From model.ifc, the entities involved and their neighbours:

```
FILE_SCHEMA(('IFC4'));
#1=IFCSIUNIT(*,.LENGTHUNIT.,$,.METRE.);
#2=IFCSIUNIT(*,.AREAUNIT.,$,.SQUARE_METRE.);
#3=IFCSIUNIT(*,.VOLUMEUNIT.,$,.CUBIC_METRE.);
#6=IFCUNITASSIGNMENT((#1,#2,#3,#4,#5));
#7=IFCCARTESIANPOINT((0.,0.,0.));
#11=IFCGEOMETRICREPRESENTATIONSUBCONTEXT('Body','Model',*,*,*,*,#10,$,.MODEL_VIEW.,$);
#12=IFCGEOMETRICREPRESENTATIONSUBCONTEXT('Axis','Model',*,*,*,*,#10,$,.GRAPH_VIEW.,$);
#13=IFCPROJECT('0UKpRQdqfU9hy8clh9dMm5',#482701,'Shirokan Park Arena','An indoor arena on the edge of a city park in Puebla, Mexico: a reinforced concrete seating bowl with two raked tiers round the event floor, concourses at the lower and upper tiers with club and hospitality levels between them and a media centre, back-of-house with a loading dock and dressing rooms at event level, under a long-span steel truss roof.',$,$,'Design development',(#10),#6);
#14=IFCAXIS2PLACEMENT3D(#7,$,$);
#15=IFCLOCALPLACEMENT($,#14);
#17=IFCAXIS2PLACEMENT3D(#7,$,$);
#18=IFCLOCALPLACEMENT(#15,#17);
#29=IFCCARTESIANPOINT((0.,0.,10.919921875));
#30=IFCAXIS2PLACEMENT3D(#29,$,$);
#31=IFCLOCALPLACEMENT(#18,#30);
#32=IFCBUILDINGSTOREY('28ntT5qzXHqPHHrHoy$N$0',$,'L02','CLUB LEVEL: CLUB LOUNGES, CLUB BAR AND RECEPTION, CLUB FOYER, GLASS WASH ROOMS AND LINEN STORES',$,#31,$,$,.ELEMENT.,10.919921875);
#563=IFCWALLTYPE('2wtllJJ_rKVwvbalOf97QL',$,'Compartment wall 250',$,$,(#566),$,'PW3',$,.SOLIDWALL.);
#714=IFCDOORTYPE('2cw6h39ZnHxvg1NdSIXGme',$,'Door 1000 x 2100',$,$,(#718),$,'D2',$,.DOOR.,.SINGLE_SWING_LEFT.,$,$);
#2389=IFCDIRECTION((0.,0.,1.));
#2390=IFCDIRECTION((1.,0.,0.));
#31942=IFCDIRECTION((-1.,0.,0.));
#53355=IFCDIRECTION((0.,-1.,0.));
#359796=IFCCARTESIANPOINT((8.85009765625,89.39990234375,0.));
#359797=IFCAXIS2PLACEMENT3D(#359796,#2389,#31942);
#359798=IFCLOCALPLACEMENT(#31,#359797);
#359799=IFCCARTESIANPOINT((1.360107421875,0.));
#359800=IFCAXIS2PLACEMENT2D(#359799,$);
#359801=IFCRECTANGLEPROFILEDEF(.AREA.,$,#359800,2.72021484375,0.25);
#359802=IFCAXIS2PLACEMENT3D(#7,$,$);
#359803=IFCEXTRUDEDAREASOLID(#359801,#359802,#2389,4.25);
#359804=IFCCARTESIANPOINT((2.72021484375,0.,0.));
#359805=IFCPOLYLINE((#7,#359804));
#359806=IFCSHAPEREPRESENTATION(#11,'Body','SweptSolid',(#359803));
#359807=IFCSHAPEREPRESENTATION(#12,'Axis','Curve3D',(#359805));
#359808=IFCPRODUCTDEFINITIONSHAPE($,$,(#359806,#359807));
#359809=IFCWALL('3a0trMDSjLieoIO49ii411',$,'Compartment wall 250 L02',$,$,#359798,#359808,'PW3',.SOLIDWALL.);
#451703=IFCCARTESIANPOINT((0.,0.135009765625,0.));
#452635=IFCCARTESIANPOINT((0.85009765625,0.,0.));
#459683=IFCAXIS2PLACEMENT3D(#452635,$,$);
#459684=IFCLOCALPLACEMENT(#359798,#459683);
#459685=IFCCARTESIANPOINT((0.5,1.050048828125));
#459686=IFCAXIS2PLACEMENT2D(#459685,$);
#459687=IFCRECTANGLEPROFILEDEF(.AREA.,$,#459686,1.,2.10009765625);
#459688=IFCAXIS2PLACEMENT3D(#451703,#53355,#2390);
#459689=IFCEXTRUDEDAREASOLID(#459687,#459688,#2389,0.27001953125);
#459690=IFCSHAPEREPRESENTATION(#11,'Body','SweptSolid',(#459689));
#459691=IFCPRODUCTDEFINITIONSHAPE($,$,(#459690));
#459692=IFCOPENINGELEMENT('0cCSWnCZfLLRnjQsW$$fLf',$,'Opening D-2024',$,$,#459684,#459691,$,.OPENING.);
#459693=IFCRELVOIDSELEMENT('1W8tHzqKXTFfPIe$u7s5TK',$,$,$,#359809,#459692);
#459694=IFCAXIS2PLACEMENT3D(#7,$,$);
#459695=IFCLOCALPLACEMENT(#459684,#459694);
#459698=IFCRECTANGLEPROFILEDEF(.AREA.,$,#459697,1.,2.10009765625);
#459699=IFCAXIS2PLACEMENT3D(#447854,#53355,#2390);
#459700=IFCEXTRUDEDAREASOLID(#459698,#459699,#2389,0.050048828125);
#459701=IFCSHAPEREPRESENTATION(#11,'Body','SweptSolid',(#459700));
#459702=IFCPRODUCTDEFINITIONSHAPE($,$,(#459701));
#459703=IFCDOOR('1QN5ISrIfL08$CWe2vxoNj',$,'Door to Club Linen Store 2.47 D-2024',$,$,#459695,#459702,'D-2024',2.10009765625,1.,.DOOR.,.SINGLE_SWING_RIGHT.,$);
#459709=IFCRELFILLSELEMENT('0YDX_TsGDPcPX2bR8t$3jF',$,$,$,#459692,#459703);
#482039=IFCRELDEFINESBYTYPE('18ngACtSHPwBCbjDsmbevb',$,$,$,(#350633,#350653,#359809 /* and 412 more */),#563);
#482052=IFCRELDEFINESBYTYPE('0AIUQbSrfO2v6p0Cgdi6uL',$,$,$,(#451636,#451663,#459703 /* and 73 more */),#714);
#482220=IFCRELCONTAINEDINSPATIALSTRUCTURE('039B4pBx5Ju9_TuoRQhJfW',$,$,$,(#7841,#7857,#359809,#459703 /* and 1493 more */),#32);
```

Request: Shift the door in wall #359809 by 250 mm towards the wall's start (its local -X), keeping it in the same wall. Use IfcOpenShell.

```python
import ifcopenshell
import ifcopenshell.api.geometry
import ifcopenshell.util.placement
import ifcopenshell.util.unit

model = ifcopenshell.open("model.ifc")
unit_scale = ifcopenshell.util.unit.calculate_unit_scale(model)

door = model.by_id(459703)
opening = door.FillsVoids[0].RelatingOpeningElement
wall = opening.VoidsElements[0].RelatingBuildingElement

wall_matrix = ifcopenshell.util.placement.get_local_placement(wall.ObjectPlacement)
shift = wall_matrix[:3, 0] * -0.25 / unit_scale
before = ifcopenshell.util.placement.get_local_placement(door.ObjectPlacement)[:3, 3].copy()

# The door is placed relative to its opening, so it follows when the opening moves.
matrix = ifcopenshell.util.placement.get_local_placement(opening.ObjectPlacement)
matrix[:3, 3] += shift
ifcopenshell.api.geometry.edit_object_placement(
    model, product=opening, matrix=matrix, is_si=False, should_transform_children=True
)

after = ifcopenshell.util.placement.get_local_placement(door.ObjectPlacement)[:3, 3]
print("door moved by", (after - before).round(3) + 0.0)

model.write("model-out.ifc")
```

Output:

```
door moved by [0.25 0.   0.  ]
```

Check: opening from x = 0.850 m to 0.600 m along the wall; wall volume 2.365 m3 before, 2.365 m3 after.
